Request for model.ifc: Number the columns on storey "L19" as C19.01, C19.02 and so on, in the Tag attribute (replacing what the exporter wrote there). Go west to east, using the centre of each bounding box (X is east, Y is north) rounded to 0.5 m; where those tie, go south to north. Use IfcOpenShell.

First a look at what the model holds.

```python
import ifcopenshell
import ifcopenshell.util.element
import ifcopenshell.util.placement

model = ifcopenshell.open("model.ifc")
print(model.schema)
storey = next(s for s in model.by_type("IfcBuildingStorey") if s.Name == "L19")
columns = [e for e in ifcopenshell.util.element.get_decomposition(storey) if e.is_a("IfcColumn")]
for e in sorted(columns, key=lambda e: e.id()):
    origin = ifcopenshell.util.placement.get_local_placement(e.ObjectPlacement)[:3, 3]
    print(e.id(), e.Tag, e.Name, origin.round(2) + 0.0, sep=" | ")
```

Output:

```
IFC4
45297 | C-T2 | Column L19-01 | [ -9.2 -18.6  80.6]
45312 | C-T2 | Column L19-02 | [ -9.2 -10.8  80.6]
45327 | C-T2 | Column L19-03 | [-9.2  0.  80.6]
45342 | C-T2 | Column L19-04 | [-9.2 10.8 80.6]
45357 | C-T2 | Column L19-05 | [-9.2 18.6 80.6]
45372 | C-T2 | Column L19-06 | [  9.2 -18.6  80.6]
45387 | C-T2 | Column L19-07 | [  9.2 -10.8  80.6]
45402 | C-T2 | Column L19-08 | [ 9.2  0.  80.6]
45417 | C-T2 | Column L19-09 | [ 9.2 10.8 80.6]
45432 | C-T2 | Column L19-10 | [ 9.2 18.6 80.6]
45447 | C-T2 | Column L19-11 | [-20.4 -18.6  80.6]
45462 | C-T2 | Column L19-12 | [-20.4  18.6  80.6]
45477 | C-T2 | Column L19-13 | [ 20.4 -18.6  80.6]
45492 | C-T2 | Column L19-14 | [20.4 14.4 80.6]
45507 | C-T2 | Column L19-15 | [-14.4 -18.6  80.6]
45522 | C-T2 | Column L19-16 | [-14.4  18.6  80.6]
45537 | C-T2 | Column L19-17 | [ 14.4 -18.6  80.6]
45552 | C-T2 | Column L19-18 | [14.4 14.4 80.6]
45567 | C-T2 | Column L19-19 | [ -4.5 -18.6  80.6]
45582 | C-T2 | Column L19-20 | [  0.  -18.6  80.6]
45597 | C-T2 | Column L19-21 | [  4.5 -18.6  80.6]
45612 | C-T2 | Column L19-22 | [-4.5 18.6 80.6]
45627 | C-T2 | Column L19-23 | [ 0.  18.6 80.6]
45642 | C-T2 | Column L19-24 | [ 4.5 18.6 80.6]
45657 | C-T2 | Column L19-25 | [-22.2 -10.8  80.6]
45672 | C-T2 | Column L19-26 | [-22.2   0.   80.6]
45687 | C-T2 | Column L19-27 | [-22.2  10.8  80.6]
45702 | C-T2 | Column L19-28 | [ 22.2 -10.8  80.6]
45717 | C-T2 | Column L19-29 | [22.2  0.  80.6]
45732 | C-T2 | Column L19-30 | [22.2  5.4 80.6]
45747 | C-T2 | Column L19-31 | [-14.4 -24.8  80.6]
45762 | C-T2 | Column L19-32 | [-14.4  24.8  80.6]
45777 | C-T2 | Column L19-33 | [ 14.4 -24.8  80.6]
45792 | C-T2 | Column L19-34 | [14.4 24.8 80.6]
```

```python
import ifcopenshell
import ifcopenshell.geom
import ifcopenshell.util.element
import ifcopenshell.util.shape

model = ifcopenshell.open("model.ifc")
settings = ifcopenshell.geom.settings()
settings.set("use-world-coords", True)


def centre(element):
    shape = ifcopenshell.geom.create_shape(settings, element)
    return ifcopenshell.util.shape.get_bbox_centroid(shape.geometry)


storey = next(s for s in model.by_type("IfcBuildingStorey") if s.Name == "L19")
columns = [e for e in ifcopenshell.util.element.get_decomposition(storey) if e.is_a("IfcColumn")]

# Insertion points can sit at a corner or the storey origin, so sort by the geometry (in metres).
centres = {e: centre(e) for e in columns}
columns.sort(key=lambda e: (round(centres[e][0] / 0.5), centres[e][1]))

for i, e in enumerate(columns, start=1):
    number = f"C19.{i:02d}"
    e.Tag = number
    print(e.id(), number)

model.write("model-out.ifc")
```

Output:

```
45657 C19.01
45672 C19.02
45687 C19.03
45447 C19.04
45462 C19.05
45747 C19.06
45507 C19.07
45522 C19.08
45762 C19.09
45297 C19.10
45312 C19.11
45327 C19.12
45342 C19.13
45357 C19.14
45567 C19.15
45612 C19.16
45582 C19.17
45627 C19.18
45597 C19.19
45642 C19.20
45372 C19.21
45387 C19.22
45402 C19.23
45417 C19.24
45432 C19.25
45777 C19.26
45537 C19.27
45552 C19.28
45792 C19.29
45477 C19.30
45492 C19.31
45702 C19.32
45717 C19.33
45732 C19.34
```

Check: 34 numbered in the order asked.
